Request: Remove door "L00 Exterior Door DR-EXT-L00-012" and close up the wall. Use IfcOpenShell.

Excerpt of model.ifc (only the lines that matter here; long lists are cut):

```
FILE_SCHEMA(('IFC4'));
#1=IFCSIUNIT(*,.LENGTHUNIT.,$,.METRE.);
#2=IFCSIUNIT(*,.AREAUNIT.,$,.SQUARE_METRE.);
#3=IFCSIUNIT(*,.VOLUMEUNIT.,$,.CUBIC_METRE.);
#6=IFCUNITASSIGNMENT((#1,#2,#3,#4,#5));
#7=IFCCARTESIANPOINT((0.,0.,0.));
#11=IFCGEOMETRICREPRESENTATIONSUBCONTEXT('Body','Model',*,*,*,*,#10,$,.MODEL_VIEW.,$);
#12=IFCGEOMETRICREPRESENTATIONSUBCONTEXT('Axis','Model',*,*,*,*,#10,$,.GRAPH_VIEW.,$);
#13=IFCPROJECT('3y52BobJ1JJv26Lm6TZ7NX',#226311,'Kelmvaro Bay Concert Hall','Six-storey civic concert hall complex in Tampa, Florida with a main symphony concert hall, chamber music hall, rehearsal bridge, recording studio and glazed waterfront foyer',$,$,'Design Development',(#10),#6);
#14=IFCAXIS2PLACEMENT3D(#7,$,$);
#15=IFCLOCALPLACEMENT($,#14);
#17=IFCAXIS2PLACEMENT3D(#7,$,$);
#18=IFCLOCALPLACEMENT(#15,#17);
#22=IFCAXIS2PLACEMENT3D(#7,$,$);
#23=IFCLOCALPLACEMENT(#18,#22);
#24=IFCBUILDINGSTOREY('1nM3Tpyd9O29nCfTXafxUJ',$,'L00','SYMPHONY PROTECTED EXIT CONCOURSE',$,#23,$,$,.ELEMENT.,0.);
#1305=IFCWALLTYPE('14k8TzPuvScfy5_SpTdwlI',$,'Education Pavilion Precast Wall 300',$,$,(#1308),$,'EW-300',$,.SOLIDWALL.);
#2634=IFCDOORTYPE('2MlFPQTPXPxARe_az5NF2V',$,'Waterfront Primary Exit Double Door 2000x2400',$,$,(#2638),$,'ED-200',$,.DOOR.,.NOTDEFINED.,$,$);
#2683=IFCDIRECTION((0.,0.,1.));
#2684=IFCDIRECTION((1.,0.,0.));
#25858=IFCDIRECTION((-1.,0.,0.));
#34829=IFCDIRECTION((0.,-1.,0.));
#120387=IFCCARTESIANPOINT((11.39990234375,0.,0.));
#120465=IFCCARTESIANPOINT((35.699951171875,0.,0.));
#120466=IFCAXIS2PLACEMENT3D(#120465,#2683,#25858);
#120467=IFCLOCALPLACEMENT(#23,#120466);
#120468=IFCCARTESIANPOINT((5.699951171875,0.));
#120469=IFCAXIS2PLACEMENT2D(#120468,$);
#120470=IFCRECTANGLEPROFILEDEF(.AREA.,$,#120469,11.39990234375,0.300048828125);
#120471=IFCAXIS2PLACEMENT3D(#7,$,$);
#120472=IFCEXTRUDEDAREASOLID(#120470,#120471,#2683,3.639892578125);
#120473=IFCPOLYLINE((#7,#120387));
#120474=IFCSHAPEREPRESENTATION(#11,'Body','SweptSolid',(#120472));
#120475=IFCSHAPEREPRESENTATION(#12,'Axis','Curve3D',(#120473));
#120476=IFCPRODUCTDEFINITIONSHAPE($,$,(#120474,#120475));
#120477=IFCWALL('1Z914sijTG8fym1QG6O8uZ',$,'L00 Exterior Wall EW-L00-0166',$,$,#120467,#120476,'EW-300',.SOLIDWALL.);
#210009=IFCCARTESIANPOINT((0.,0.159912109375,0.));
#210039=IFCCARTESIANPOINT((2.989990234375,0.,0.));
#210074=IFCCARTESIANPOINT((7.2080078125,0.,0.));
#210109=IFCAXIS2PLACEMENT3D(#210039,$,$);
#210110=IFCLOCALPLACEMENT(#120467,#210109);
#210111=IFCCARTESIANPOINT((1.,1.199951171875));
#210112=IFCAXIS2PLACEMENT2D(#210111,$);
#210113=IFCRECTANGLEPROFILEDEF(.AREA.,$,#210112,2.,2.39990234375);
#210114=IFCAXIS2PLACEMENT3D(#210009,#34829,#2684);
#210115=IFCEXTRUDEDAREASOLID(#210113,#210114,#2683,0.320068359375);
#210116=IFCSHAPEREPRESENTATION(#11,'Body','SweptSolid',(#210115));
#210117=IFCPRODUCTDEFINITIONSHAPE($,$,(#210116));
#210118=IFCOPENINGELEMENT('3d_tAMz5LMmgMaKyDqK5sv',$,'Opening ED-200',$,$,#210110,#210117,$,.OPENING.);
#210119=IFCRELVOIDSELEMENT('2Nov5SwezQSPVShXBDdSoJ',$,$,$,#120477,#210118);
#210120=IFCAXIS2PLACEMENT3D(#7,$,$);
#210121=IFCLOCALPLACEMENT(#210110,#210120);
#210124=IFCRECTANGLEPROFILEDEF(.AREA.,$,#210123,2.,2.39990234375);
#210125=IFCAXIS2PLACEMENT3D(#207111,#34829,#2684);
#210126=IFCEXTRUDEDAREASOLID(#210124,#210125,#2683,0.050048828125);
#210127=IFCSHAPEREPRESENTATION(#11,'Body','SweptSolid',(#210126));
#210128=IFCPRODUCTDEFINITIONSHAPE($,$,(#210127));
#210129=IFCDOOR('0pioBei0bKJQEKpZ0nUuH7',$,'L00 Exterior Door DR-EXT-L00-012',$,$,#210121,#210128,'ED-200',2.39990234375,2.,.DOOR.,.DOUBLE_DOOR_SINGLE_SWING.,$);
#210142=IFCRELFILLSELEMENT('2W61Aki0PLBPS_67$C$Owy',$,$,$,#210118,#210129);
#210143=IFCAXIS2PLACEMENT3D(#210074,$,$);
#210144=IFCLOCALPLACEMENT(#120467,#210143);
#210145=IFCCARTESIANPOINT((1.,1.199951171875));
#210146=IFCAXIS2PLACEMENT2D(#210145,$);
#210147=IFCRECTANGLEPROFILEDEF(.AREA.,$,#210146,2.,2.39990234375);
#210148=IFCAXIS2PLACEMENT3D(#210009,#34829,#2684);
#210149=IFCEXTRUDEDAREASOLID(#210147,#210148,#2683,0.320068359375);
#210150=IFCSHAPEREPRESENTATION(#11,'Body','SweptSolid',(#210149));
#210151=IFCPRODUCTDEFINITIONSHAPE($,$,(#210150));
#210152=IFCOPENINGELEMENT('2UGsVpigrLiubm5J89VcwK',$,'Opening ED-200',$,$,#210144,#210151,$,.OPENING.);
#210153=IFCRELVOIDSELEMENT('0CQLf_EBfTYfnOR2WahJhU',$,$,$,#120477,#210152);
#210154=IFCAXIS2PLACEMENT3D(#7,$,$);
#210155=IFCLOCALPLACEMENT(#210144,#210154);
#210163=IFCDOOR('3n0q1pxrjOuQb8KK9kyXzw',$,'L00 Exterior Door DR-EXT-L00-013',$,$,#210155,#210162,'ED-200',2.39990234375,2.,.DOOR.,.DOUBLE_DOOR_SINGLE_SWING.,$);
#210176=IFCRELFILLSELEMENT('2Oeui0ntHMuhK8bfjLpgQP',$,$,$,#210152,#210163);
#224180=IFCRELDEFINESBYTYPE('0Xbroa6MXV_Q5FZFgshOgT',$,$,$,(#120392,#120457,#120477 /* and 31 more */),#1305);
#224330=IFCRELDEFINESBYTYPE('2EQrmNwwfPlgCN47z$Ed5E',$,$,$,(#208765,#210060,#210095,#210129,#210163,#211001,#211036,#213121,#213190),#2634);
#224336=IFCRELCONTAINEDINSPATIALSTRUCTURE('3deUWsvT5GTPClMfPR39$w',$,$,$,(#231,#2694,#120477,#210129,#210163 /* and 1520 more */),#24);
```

```python
import ifcopenshell
import ifcopenshell.api.feature
import ifcopenshell.api.root
import ifcopenshell.geom
import ifcopenshell.util.shape

model = ifcopenshell.open("model.ifc")
settings = ifcopenshell.geom.settings()


def volume(element):
    """Net volume in cubic metres, openings subtracted."""
    shape = ifcopenshell.geom.create_shape(settings, element)
    return ifcopenshell.util.shape.get_volume(shape.geometry)


door = model.by_guid("0pioBei0bKJQEKpZ0nUuH7")
opening = door.FillsVoids[0].RelatingOpeningElement
wall = opening.VoidsElements[0].RelatingBuildingElement
before = volume(wall)

ifcopenshell.api.root.remove_product(model, product=door)
ifcopenshell.api.feature.remove_feature(model, feature=opening)

after = volume(wall)

print(f"wall volume {before:.3f} -> {after:.3f} m3")

model.write("model_edited.ifc")
```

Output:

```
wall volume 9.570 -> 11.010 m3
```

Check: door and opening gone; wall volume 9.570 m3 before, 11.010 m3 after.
